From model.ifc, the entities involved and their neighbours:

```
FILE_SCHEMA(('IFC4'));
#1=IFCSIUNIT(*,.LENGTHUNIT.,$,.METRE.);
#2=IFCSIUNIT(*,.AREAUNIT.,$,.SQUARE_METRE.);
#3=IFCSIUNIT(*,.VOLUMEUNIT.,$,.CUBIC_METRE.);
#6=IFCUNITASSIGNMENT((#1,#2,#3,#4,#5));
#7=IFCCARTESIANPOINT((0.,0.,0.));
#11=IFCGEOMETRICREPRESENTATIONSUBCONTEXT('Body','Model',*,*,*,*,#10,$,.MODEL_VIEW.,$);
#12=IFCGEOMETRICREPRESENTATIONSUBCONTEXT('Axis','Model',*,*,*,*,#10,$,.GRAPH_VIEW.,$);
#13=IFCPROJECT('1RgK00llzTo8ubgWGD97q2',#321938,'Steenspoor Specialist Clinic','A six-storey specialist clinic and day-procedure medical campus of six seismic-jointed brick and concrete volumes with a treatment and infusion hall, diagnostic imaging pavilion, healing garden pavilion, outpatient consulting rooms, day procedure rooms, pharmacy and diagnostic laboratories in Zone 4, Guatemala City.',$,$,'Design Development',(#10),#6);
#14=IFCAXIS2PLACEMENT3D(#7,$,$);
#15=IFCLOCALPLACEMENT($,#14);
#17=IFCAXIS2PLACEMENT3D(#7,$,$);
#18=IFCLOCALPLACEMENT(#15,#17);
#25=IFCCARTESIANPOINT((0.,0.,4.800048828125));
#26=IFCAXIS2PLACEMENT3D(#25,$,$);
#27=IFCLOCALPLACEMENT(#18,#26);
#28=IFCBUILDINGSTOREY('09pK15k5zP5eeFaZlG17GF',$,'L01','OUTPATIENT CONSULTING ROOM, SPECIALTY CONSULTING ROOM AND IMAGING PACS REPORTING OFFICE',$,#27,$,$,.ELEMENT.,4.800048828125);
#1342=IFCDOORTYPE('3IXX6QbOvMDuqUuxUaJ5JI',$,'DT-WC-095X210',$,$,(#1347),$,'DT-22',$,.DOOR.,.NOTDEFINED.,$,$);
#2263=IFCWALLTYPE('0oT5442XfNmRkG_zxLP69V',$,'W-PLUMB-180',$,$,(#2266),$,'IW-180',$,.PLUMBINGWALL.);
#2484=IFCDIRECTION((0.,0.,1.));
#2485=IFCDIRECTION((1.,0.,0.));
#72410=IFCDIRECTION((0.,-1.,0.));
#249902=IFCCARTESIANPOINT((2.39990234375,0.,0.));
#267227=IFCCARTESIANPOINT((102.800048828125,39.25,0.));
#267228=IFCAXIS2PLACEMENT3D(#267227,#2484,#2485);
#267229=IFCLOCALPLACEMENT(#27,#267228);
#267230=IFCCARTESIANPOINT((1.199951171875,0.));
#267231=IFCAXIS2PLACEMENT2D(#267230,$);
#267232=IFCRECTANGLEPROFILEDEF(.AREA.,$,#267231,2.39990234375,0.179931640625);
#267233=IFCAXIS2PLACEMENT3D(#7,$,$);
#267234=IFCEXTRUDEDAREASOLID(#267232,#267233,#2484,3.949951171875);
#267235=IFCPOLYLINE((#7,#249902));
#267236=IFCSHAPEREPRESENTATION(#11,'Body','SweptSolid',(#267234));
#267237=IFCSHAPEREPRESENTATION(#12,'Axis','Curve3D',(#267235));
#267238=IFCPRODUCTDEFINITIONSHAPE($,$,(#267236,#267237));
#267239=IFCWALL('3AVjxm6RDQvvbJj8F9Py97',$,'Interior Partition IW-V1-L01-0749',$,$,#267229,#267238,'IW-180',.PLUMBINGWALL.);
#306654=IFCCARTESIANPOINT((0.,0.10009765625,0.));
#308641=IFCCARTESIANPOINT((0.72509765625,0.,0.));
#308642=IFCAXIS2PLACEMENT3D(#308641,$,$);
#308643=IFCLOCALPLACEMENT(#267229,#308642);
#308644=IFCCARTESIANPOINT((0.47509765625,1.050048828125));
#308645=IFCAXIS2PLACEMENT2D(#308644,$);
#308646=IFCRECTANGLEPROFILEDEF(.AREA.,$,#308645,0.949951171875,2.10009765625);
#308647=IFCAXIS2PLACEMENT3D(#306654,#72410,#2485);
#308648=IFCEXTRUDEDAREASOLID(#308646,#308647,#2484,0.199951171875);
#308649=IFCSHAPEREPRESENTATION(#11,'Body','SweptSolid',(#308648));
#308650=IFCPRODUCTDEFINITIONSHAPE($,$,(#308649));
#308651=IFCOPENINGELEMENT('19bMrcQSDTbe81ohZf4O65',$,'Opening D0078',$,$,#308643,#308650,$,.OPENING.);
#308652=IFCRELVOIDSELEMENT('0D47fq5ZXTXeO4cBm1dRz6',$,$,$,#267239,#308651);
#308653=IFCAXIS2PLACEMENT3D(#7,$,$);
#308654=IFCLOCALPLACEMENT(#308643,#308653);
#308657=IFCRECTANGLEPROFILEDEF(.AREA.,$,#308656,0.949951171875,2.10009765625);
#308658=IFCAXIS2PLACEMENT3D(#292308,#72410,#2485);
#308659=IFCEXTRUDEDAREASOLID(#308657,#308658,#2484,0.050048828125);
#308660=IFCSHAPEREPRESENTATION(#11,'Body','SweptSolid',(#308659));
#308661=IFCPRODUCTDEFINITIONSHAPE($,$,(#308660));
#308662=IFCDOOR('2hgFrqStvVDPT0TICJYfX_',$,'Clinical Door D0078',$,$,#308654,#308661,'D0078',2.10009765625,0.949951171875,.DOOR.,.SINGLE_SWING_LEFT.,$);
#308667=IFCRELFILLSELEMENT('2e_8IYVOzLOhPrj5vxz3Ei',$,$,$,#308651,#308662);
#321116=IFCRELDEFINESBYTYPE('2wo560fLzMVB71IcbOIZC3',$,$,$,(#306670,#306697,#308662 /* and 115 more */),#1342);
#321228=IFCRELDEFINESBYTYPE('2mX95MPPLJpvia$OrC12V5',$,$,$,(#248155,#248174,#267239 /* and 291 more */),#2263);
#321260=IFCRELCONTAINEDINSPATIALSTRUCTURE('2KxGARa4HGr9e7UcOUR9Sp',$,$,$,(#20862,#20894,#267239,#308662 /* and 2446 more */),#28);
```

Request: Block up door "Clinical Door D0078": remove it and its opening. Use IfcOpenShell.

```python
import ifcopenshell
import ifcopenshell.api.feature
import ifcopenshell.api.root
import ifcopenshell.geom
import ifcopenshell.util.shape

model = ifcopenshell.open("model.ifc")
settings = ifcopenshell.geom.settings()


def volume(element):
    """Net volume in cubic metres, openings subtracted."""
    shape = ifcopenshell.geom.create_shape(settings, element)
    return ifcopenshell.util.shape.get_volume(shape.geometry)


door = model.by_guid("2hgFrqStvVDPT0TICJYfX_")
opening = door.FillsVoids[0].RelatingOpeningElement
wall = opening.VoidsElements[0].RelatingBuildingElement
before = volume(wall)

ifcopenshell.api.root.remove_product(model, product=door)
ifcopenshell.api.feature.remove_feature(model, feature=opening)

after = volume(wall)

print(f"wall volume {before:.3f} -> {after:.3f} m3")

model.write("model_rev.ifc")
```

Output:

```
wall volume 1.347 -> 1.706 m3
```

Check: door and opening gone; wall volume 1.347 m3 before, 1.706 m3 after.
